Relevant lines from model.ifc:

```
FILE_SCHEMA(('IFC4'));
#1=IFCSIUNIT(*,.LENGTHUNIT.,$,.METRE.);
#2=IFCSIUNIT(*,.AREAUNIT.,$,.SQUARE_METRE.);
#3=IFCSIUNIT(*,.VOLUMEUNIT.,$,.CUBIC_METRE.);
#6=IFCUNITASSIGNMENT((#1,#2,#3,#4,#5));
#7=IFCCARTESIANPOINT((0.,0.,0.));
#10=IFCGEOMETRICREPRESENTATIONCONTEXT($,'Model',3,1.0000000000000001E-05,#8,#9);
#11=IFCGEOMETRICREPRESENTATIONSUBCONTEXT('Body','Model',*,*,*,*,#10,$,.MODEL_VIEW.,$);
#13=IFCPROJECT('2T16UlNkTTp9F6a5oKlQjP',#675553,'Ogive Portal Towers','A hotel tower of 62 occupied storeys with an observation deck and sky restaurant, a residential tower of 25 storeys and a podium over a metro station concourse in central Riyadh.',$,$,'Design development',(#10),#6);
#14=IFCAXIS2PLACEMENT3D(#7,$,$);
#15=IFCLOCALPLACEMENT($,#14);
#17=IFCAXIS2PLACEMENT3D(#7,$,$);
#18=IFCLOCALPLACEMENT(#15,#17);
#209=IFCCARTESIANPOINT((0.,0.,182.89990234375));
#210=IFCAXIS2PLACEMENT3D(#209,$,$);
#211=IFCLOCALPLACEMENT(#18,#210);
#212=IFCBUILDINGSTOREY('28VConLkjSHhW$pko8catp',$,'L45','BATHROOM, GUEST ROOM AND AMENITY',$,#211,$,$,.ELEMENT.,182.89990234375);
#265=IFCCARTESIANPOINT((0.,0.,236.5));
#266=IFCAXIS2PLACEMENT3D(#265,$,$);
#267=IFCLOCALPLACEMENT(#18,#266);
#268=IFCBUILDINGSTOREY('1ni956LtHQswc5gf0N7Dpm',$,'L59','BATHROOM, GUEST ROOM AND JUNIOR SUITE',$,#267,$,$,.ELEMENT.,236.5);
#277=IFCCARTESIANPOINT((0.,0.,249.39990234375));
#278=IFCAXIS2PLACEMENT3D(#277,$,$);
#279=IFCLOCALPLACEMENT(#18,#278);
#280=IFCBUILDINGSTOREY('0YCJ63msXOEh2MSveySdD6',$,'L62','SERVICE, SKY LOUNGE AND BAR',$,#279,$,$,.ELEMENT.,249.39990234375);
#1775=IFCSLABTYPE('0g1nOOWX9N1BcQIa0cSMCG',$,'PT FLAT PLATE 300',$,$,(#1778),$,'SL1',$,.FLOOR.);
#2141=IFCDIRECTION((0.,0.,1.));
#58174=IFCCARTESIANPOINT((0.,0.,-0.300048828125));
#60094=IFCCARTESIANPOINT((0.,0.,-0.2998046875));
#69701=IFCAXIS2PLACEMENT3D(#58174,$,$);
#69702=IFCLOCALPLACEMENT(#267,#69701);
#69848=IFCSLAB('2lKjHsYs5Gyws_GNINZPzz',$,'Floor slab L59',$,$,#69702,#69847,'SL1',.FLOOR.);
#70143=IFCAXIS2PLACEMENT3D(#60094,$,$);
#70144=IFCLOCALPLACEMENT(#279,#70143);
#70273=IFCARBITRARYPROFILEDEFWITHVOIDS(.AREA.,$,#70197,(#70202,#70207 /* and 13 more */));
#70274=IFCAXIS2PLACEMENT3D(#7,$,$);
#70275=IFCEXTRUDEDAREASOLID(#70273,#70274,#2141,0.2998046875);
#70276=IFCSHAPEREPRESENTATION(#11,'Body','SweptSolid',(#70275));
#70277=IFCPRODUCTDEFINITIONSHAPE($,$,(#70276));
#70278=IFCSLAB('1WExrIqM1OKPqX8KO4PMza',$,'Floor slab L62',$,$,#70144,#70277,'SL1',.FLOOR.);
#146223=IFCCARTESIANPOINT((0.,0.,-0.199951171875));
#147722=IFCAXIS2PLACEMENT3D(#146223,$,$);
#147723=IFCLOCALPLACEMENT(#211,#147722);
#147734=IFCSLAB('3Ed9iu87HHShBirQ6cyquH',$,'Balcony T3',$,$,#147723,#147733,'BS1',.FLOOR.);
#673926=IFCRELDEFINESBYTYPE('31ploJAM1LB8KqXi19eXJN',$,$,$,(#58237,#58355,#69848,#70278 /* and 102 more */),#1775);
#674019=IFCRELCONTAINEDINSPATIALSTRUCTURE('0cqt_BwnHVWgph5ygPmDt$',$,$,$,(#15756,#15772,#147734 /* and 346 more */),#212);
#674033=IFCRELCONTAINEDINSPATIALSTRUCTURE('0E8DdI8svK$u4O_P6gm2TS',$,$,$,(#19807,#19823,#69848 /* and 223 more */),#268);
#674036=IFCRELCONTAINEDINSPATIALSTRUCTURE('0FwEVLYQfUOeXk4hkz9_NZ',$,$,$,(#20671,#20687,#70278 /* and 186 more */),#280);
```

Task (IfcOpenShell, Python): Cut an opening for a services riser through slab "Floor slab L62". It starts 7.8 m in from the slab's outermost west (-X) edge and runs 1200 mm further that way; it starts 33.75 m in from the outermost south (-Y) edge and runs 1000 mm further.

```python
import numpy as np
import ifcopenshell
import ifcopenshell.api.feature
import ifcopenshell.api.geometry
import ifcopenshell.api.root
import ifcopenshell.geom
import ifcopenshell.util.placement
import ifcopenshell.util.representation
import ifcopenshell.util.shape
import ifcopenshell.util.unit

model = ifcopenshell.open("model.ifc")
unit_scale = ifcopenshell.util.unit.calculate_unit_scale(model)
settings = ifcopenshell.geom.settings()


def volume(element):
    """Net volume in cubic metres, openings subtracted."""
    shape = ifcopenshell.geom.create_shape(settings, element)
    return ifcopenshell.util.shape.get_volume(shape.geometry)


slab = model.by_guid("1WExrIqM1OKPqX8KO4PMza")
before = volume(slab)

# Extent in the slab's own axes, in metres. The edges named are its -X and -Y sides.
slab_shape = ifcopenshell.geom.create_shape(settings, slab)
vertices = ifcopenshell.util.shape.get_vertices(slab_shape.geometry)
x_min, y_min, bottom = vertices.min(axis=0)
top = vertices[:, 2].max()

opening = ifcopenshell.api.root.create_entity(model, ifc_class="IfcOpeningElement", name="Services riser opening", predefined_type="OPENING")
context = ifcopenshell.util.representation.get_context(model, "Model", "Body", "MODEL_VIEW")
width, depth = 1.2, 1
outline = [(0.0, 0.0), (width, 0.0), (width, depth), (0.0, depth), (0.0, 0.0)]
# Overshoot both faces by 50 mm so the cut is clean.
shape = ifcopenshell.api.geometry.add_slab_representation(
    model, context=context, depth=top - bottom + 0.1, polyline=outline
)
ifcopenshell.api.geometry.assign_representation(model, product=opening, representation=shape)

matrix = ifcopenshell.util.placement.get_local_placement(slab.ObjectPlacement)
matrix[:, 3] = matrix @ np.append(np.array([x_min + 7.8, y_min + 33.75, bottom - 0.05]) / unit_scale, 1.0)
ifcopenshell.api.geometry.edit_object_placement(model, product=opening, matrix=matrix, is_si=False)
ifcopenshell.api.feature.add_feature(model, feature=opening, element=slab)

after = volume(slab)

print(f"slab volume {before:.3f} -> {after:.3f} m3")

model.write("model_rev.ifc")
```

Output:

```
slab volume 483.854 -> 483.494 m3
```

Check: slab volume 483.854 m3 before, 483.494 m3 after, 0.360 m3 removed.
